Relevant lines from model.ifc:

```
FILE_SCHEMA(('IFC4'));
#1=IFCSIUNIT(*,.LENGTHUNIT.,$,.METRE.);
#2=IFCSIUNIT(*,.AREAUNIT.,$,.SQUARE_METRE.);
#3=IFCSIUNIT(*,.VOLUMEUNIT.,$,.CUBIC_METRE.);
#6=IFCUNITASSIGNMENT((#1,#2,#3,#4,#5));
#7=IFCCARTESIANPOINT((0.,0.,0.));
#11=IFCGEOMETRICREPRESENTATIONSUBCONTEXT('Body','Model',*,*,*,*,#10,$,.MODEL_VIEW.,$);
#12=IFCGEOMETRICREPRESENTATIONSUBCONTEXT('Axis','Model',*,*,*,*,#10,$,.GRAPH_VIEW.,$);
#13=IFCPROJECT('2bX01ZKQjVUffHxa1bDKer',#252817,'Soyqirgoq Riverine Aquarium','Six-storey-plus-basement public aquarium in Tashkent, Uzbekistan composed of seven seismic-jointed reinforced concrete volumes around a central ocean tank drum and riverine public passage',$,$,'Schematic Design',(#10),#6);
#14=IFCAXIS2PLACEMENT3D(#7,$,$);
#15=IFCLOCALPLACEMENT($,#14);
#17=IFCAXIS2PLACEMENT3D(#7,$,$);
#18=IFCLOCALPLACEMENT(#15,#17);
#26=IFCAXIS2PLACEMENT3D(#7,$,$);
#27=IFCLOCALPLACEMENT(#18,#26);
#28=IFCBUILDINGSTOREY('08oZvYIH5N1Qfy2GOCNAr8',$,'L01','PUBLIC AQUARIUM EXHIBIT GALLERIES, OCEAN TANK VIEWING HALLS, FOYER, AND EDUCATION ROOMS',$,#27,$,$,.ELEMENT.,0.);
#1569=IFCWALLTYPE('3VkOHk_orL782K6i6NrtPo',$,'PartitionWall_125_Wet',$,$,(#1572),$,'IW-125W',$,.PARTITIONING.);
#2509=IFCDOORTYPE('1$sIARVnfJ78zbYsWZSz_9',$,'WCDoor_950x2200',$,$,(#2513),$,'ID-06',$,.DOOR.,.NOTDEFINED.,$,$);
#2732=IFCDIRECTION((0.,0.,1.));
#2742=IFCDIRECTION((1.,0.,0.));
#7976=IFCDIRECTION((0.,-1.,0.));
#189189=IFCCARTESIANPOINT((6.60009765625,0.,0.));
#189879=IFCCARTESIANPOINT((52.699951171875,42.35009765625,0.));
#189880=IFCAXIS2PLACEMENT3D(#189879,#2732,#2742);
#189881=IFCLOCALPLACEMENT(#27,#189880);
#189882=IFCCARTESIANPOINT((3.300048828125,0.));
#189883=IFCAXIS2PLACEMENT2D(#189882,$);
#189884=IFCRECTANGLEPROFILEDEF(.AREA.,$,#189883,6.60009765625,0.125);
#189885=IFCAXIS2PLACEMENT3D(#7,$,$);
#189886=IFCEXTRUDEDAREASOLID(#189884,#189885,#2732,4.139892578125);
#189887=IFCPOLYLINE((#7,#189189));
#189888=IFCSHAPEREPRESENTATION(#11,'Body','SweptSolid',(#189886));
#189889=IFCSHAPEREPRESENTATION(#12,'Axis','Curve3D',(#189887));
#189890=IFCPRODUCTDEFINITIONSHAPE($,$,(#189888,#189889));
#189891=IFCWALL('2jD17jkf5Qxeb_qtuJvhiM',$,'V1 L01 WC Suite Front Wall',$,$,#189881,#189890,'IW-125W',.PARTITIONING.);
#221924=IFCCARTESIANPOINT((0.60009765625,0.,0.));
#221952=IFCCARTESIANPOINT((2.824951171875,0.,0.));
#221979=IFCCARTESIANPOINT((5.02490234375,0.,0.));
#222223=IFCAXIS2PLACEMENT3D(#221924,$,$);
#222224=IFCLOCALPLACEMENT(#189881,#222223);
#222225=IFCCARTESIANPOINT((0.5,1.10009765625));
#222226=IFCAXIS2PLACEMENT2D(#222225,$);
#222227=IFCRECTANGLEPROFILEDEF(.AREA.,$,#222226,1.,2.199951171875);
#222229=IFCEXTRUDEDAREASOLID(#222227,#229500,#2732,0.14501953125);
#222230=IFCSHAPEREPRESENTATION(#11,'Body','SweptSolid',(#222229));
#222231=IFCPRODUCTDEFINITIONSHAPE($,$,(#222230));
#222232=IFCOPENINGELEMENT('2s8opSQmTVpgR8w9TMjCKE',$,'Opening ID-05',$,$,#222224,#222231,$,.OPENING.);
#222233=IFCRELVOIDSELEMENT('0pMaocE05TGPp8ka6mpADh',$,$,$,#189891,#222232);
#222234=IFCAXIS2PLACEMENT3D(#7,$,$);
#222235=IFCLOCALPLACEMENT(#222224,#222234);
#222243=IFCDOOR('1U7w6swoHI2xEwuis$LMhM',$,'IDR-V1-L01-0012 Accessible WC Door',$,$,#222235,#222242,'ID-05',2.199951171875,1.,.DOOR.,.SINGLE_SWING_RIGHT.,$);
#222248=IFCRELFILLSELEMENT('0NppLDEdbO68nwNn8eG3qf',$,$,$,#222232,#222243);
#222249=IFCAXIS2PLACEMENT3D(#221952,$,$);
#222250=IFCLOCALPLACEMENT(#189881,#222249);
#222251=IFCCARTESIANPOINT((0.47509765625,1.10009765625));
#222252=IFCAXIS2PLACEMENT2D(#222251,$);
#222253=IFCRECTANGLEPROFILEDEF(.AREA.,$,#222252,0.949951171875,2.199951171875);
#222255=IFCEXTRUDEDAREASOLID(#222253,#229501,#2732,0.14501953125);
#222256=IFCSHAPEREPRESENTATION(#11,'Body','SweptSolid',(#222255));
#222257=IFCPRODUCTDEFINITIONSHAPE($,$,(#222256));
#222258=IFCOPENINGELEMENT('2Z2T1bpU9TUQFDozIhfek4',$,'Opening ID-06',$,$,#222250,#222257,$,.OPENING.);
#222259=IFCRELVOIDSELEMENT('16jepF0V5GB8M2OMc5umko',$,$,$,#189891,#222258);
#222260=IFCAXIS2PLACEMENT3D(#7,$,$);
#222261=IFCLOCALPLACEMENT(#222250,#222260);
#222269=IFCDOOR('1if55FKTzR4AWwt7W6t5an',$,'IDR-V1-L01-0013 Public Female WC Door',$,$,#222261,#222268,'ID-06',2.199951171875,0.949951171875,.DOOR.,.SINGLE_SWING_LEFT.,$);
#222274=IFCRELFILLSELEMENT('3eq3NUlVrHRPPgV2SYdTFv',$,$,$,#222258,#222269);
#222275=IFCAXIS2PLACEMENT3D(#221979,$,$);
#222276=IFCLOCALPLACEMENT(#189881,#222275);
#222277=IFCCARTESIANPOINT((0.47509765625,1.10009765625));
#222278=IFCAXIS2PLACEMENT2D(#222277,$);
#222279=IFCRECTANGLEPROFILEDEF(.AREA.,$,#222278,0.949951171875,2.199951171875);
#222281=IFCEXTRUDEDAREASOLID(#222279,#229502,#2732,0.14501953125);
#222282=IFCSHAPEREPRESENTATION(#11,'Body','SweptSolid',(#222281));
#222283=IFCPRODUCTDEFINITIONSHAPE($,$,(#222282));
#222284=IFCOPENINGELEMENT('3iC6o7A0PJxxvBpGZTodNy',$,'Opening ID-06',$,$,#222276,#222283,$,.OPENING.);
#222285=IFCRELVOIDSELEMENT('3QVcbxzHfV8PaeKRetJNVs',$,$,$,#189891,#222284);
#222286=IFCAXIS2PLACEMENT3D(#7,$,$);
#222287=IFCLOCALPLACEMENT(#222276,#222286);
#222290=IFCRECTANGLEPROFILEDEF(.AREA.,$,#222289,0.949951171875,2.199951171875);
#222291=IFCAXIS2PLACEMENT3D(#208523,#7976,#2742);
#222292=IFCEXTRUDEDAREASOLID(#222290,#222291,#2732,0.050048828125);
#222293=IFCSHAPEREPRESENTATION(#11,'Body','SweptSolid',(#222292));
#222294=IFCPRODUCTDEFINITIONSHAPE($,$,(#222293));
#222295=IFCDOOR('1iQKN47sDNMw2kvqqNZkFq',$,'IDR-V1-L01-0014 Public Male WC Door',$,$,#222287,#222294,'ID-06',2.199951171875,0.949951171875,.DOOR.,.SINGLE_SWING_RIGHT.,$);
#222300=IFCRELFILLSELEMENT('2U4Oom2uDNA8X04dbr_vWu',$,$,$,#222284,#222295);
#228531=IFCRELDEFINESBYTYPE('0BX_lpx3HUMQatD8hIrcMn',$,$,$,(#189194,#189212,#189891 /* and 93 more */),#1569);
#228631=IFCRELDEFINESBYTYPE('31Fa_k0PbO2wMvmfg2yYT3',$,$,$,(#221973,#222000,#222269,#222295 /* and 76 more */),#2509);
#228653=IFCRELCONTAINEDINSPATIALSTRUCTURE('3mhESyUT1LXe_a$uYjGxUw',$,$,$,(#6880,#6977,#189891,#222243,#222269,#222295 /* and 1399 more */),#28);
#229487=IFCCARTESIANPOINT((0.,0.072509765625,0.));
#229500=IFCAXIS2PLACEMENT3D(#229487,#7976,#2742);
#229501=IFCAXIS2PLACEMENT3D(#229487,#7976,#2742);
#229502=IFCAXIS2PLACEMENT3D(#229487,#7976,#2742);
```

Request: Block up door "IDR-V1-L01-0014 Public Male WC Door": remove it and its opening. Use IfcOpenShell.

```python
import ifcopenshell
import ifcopenshell.api.feature
import ifcopenshell.api.root
import ifcopenshell.geom
import ifcopenshell.util.shape

model = ifcopenshell.open("model.ifc")
settings = ifcopenshell.geom.settings()


def volume(element):
    """Net volume in cubic metres, openings subtracted."""
    shape = ifcopenshell.geom.create_shape(settings, element)
    return ifcopenshell.util.shape.get_volume(shape.geometry)


door = model.by_id(222295)
opening = door.FillsVoids[0].RelatingOpeningElement
wall = opening.VoidsElements[0].RelatingBuildingElement
before = volume(wall)

ifcopenshell.api.root.remove_product(model, product=door)
ifcopenshell.api.feature.remove_feature(model, feature=opening)

after = volume(wall)

print(f"wall volume {before:.3f} -> {after:.3f} m3")

model.write("model_edited.ifc")
```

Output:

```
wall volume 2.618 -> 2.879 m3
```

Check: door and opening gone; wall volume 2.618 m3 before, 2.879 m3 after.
